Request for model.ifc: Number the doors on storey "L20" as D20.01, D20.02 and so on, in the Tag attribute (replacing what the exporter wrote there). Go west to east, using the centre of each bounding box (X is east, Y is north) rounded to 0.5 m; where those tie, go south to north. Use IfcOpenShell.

First a look at what the model holds.

```python
import ifcopenshell
import ifcopenshell.util.element
import ifcopenshell.util.placement

model = ifcopenshell.open("model.ifc")
print(model.schema)
storey = next(s for s in model.by_type("IfcBuildingStorey") if s.Name == "L20")
doors = [e for e in ifcopenshell.util.element.get_decomposition(storey) if e.is_a("IfcDoor")]
for e in sorted(doors, key=lambda e: e.id()):
    origin = ifcopenshell.util.placement.get_local_placement(e.ObjectPlacement)[:3, 3]
    print(e.id(), e.Tag, e.Name, origin.round(2) + 0.0, sep=" | ")
```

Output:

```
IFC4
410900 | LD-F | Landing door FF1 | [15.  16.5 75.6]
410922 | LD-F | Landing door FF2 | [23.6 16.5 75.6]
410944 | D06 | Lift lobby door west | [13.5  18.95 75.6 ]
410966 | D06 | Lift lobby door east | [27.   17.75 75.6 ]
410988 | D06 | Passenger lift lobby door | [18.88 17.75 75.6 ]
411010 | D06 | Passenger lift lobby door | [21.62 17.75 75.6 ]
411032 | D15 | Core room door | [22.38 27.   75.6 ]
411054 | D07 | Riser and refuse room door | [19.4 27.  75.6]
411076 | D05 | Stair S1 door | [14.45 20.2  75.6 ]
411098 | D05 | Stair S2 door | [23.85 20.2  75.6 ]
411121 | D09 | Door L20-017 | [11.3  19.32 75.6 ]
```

```python
import ifcopenshell
import ifcopenshell.geom
import ifcopenshell.util.element
import ifcopenshell.util.shape

model = ifcopenshell.open("model.ifc")
settings = ifcopenshell.geom.settings()
settings.set("use-world-coords", True)


def centre(element):
    shape = ifcopenshell.geom.create_shape(settings, element)
    return ifcopenshell.util.shape.get_bbox_centroid(shape.geometry)


storey = next(s for s in model.by_type("IfcBuildingStorey") if s.Name == "L20")
doors = [e for e in ifcopenshell.util.element.get_decomposition(storey) if e.is_a("IfcDoor")]

# Insertion points can sit at a corner or the storey origin, so sort by the geometry (in metres).
centres = {e: centre(e) for e in doors}
doors.sort(key=lambda e: (round(centres[e][0] / 0.5), centres[e][1]))

for i, e in enumerate(doors, start=1):
    number = f"D20.{i:02d}"
    e.Tag = number
    print(e.id(), number)

model.write("model_rev.ifc")
```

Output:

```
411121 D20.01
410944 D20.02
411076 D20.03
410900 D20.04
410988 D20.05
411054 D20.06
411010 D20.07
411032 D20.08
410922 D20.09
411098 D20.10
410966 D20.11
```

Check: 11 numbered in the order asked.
